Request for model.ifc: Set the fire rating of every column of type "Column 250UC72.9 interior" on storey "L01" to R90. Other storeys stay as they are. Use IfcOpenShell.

First a look at what the model holds.

```python
import ifcopenshell
import ifcopenshell.util.element

model = ifcopenshell.open("model.ifc")
print(model.schema)
storey = next(s for s in model.by_type("IfcBuildingStorey") if s.Name == "L01")
columns = [e for e in ifcopenshell.util.element.get_decomposition(storey) if e.is_a("IfcColumn")]
seen = {}
for e in columns:
    element_type = ifcopenshell.util.element.get_type(e)
    key = (element_type.Name if element_type != e and element_type else None, ifcopenshell.util.element.get_pset(e, "Pset_ColumnCommon", "FireRating"))
    seen[key] = seen.get(key, 0) + 1
for (name, value), count in sorted(seen.items(), key=str):
    print(count, "x", name, "|", value)
```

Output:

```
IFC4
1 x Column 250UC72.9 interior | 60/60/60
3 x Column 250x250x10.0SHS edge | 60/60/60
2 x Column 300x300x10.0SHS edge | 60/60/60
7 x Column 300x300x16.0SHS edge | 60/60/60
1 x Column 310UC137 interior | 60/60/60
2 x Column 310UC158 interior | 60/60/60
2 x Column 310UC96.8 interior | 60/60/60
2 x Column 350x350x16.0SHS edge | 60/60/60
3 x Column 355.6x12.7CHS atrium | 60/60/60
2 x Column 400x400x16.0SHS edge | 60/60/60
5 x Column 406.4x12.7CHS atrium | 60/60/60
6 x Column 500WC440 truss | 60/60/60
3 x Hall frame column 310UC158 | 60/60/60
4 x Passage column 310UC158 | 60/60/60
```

```python
import ifcopenshell
import ifcopenshell.api.pset
import ifcopenshell.util.element

model = ifcopenshell.open("model.ifc")

storey = next(s for s in model.by_type("IfcBuildingStorey") if s.Name == "L01")
columns = [e for e in ifcopenshell.util.element.get_decomposition(storey) if e.is_a("IfcColumn")]

count = 0
for e in columns:
    element_type = ifcopenshell.util.element.get_type(e)
    if element_type in (None, e) or element_type.Name != "Column 250UC72.9 interior":
        continue
    # add_pset returns the element's existing set when there is one.
    pset = ifcopenshell.api.pset.add_pset(model, product=e, name="Pset_ColumnCommon")
    ifcopenshell.api.pset.edit_pset(model, pset=pset, properties={"FireRating": "R90"})
    count += 1

print(count, "columns updated")

model.write("model_rev.ifc")
```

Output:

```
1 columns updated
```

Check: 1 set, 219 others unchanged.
